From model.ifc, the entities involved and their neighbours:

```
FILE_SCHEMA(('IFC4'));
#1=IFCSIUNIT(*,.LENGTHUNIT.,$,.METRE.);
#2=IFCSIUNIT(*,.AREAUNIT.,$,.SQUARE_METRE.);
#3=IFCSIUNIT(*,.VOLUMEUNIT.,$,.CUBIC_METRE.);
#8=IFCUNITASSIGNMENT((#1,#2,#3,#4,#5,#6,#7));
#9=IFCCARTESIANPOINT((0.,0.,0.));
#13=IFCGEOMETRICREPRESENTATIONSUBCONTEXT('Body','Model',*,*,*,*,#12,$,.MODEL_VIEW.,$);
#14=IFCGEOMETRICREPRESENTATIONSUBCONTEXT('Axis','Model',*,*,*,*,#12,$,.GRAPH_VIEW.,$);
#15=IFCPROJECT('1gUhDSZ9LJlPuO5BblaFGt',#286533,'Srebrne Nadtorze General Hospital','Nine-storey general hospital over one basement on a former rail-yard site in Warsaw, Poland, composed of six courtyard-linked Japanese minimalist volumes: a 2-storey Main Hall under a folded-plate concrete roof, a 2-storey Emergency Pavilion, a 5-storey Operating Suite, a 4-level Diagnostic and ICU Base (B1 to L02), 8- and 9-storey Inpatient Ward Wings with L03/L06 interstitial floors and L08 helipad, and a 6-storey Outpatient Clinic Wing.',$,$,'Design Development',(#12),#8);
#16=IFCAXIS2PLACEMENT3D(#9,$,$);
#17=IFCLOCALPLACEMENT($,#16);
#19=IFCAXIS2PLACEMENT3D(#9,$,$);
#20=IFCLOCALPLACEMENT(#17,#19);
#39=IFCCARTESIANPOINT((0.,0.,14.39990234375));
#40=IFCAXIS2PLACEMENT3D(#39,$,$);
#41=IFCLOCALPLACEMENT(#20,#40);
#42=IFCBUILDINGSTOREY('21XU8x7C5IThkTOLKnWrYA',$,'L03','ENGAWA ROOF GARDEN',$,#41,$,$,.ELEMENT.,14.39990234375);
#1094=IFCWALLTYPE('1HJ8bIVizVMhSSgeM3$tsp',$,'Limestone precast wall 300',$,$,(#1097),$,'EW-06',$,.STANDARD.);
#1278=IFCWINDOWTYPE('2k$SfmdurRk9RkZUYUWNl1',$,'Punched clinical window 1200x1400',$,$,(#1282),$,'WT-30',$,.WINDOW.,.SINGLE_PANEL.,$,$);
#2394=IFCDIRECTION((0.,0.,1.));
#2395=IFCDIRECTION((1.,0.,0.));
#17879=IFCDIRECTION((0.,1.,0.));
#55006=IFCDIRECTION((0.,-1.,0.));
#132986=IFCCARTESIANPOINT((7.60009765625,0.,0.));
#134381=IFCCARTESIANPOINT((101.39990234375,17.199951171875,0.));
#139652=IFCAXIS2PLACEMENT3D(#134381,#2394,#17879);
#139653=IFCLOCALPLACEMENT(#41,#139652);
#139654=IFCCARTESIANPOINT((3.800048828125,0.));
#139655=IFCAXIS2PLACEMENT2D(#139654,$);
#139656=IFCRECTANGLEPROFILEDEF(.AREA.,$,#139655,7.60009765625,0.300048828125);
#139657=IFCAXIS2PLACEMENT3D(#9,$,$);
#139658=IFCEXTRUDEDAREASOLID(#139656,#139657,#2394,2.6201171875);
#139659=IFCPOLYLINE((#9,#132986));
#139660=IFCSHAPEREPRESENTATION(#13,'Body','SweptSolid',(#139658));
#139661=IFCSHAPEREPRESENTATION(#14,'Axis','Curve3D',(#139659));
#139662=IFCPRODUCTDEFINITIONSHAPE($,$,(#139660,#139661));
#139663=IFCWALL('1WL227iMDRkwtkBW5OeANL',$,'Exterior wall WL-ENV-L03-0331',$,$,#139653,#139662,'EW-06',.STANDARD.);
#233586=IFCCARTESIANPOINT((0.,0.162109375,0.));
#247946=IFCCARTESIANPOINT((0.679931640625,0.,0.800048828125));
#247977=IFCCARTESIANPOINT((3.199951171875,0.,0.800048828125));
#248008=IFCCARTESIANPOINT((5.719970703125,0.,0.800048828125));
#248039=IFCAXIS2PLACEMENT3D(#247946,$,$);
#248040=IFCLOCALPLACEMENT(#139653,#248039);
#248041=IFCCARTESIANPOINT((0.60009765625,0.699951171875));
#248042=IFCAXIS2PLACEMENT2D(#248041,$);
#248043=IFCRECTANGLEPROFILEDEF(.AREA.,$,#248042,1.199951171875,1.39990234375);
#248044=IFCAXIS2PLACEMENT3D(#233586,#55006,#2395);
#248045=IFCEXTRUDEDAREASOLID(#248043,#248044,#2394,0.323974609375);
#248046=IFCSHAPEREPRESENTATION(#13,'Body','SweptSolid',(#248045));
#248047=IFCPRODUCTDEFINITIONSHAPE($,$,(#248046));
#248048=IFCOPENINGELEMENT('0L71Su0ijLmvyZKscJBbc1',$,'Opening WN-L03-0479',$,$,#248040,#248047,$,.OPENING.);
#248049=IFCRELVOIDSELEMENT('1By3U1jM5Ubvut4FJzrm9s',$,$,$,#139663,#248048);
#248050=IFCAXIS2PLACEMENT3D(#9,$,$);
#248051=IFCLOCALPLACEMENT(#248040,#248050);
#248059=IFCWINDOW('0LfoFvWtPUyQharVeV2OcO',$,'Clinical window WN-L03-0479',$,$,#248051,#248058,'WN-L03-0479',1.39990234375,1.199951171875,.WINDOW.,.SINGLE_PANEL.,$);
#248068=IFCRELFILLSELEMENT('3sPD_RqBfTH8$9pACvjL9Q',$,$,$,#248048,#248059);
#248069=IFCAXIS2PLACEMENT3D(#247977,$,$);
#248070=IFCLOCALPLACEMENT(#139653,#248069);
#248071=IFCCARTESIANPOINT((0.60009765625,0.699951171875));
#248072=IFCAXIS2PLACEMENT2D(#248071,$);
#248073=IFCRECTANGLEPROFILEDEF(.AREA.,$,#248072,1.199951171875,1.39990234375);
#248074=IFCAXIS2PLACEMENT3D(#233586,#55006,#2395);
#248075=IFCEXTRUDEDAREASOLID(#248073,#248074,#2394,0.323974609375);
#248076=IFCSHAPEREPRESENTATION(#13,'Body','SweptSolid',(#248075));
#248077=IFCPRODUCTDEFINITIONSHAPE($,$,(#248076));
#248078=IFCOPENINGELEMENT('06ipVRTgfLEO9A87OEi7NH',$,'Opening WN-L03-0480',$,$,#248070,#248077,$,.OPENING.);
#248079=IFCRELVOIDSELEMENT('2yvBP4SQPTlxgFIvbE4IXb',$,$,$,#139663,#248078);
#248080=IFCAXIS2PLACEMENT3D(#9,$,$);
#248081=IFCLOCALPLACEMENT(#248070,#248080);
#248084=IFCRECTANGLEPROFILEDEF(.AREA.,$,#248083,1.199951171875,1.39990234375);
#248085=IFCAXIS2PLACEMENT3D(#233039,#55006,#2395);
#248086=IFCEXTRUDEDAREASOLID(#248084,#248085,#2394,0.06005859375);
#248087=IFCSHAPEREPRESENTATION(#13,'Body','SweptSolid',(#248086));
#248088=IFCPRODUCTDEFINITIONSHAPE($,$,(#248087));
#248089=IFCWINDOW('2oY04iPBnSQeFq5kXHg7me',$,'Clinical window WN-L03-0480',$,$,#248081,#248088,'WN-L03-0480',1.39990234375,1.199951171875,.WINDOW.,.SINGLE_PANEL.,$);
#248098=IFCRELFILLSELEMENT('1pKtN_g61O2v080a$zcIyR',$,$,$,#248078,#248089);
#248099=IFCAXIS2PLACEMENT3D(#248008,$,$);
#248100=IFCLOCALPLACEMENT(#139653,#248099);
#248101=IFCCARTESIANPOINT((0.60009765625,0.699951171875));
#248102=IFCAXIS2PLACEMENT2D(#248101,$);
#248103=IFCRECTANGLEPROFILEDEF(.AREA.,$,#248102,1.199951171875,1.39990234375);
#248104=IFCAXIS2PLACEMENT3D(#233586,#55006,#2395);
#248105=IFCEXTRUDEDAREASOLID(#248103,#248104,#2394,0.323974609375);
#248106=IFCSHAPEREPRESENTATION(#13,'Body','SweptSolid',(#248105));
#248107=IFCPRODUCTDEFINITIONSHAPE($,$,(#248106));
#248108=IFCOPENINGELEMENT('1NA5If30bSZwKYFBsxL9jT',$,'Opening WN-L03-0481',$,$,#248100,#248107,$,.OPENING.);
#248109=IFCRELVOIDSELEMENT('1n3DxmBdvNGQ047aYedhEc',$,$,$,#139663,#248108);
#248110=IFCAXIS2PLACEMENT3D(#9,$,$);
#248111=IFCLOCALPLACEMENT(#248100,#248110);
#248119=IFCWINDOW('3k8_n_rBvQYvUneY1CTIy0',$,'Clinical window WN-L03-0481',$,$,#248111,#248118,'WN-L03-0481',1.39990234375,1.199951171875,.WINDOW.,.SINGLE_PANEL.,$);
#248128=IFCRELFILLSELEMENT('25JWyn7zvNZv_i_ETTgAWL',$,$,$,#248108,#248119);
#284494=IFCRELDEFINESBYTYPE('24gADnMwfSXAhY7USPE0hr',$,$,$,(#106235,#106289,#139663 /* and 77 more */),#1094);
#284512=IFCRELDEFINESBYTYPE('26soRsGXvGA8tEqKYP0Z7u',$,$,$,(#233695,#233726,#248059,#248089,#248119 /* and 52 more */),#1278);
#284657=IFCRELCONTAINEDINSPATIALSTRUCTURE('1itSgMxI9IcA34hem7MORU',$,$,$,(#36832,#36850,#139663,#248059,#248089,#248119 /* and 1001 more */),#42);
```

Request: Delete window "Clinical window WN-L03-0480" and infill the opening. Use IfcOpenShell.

```python
import ifcopenshell
import ifcopenshell.api.feature
import ifcopenshell.api.root
import ifcopenshell.geom
import ifcopenshell.util.shape

model = ifcopenshell.open("model.ifc")
settings = ifcopenshell.geom.settings()


def volume(element):
    """Net volume in cubic metres, openings subtracted."""
    shape = ifcopenshell.geom.create_shape(settings, element)
    return ifcopenshell.util.shape.get_volume(shape.geometry)


window = model.by_id(248089)
opening = window.FillsVoids[0].RelatingOpeningElement
wall = opening.VoidsElements[0].RelatingBuildingElement
before = volume(wall)

ifcopenshell.api.root.remove_product(model, product=window)
ifcopenshell.api.feature.remove_feature(model, feature=opening)

after = volume(wall)

print(f"wall volume {before:.3f} -> {after:.3f} m3")

model.write("model_rev.ifc")
```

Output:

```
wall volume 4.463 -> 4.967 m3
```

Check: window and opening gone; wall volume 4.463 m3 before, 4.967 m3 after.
